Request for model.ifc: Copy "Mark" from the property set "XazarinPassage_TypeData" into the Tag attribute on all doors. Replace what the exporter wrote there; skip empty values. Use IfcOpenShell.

First a look at what the model holds.

```python
import ifcopenshell
import ifcopenshell.util.element

model = ifcopenshell.open("model.ifc")
print(model.schema)
doors = model.by_type("IfcDoor")
print(len(doors), "doors")
for e in doors[:8]:
    source = ifcopenshell.util.element.get_pset(e, "XazarinPassage_TypeData", "Mark")
    target = e.Tag
    print(e.id(), repr(source), repr(target), sep=" | ")
```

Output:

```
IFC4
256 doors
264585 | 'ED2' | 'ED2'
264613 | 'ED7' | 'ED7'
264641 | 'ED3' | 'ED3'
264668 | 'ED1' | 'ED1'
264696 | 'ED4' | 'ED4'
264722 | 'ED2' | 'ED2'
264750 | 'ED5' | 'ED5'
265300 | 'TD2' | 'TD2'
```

```python
import ifcopenshell
import ifcopenshell.util.element

model = ifcopenshell.open("model.ifc")

count = 0
for e in model.by_type("IfcDoor"):
    value = ifcopenshell.util.element.get_pset(e, "XazarinPassage_TypeData", "Mark")
    current = e.Tag
    if not value or not value.strip() or current == value:
        continue
    e.Tag = value
    count += 1

print(count, "doors updated")

model.write("model-out.ifc")
```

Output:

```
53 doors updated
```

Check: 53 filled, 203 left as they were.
